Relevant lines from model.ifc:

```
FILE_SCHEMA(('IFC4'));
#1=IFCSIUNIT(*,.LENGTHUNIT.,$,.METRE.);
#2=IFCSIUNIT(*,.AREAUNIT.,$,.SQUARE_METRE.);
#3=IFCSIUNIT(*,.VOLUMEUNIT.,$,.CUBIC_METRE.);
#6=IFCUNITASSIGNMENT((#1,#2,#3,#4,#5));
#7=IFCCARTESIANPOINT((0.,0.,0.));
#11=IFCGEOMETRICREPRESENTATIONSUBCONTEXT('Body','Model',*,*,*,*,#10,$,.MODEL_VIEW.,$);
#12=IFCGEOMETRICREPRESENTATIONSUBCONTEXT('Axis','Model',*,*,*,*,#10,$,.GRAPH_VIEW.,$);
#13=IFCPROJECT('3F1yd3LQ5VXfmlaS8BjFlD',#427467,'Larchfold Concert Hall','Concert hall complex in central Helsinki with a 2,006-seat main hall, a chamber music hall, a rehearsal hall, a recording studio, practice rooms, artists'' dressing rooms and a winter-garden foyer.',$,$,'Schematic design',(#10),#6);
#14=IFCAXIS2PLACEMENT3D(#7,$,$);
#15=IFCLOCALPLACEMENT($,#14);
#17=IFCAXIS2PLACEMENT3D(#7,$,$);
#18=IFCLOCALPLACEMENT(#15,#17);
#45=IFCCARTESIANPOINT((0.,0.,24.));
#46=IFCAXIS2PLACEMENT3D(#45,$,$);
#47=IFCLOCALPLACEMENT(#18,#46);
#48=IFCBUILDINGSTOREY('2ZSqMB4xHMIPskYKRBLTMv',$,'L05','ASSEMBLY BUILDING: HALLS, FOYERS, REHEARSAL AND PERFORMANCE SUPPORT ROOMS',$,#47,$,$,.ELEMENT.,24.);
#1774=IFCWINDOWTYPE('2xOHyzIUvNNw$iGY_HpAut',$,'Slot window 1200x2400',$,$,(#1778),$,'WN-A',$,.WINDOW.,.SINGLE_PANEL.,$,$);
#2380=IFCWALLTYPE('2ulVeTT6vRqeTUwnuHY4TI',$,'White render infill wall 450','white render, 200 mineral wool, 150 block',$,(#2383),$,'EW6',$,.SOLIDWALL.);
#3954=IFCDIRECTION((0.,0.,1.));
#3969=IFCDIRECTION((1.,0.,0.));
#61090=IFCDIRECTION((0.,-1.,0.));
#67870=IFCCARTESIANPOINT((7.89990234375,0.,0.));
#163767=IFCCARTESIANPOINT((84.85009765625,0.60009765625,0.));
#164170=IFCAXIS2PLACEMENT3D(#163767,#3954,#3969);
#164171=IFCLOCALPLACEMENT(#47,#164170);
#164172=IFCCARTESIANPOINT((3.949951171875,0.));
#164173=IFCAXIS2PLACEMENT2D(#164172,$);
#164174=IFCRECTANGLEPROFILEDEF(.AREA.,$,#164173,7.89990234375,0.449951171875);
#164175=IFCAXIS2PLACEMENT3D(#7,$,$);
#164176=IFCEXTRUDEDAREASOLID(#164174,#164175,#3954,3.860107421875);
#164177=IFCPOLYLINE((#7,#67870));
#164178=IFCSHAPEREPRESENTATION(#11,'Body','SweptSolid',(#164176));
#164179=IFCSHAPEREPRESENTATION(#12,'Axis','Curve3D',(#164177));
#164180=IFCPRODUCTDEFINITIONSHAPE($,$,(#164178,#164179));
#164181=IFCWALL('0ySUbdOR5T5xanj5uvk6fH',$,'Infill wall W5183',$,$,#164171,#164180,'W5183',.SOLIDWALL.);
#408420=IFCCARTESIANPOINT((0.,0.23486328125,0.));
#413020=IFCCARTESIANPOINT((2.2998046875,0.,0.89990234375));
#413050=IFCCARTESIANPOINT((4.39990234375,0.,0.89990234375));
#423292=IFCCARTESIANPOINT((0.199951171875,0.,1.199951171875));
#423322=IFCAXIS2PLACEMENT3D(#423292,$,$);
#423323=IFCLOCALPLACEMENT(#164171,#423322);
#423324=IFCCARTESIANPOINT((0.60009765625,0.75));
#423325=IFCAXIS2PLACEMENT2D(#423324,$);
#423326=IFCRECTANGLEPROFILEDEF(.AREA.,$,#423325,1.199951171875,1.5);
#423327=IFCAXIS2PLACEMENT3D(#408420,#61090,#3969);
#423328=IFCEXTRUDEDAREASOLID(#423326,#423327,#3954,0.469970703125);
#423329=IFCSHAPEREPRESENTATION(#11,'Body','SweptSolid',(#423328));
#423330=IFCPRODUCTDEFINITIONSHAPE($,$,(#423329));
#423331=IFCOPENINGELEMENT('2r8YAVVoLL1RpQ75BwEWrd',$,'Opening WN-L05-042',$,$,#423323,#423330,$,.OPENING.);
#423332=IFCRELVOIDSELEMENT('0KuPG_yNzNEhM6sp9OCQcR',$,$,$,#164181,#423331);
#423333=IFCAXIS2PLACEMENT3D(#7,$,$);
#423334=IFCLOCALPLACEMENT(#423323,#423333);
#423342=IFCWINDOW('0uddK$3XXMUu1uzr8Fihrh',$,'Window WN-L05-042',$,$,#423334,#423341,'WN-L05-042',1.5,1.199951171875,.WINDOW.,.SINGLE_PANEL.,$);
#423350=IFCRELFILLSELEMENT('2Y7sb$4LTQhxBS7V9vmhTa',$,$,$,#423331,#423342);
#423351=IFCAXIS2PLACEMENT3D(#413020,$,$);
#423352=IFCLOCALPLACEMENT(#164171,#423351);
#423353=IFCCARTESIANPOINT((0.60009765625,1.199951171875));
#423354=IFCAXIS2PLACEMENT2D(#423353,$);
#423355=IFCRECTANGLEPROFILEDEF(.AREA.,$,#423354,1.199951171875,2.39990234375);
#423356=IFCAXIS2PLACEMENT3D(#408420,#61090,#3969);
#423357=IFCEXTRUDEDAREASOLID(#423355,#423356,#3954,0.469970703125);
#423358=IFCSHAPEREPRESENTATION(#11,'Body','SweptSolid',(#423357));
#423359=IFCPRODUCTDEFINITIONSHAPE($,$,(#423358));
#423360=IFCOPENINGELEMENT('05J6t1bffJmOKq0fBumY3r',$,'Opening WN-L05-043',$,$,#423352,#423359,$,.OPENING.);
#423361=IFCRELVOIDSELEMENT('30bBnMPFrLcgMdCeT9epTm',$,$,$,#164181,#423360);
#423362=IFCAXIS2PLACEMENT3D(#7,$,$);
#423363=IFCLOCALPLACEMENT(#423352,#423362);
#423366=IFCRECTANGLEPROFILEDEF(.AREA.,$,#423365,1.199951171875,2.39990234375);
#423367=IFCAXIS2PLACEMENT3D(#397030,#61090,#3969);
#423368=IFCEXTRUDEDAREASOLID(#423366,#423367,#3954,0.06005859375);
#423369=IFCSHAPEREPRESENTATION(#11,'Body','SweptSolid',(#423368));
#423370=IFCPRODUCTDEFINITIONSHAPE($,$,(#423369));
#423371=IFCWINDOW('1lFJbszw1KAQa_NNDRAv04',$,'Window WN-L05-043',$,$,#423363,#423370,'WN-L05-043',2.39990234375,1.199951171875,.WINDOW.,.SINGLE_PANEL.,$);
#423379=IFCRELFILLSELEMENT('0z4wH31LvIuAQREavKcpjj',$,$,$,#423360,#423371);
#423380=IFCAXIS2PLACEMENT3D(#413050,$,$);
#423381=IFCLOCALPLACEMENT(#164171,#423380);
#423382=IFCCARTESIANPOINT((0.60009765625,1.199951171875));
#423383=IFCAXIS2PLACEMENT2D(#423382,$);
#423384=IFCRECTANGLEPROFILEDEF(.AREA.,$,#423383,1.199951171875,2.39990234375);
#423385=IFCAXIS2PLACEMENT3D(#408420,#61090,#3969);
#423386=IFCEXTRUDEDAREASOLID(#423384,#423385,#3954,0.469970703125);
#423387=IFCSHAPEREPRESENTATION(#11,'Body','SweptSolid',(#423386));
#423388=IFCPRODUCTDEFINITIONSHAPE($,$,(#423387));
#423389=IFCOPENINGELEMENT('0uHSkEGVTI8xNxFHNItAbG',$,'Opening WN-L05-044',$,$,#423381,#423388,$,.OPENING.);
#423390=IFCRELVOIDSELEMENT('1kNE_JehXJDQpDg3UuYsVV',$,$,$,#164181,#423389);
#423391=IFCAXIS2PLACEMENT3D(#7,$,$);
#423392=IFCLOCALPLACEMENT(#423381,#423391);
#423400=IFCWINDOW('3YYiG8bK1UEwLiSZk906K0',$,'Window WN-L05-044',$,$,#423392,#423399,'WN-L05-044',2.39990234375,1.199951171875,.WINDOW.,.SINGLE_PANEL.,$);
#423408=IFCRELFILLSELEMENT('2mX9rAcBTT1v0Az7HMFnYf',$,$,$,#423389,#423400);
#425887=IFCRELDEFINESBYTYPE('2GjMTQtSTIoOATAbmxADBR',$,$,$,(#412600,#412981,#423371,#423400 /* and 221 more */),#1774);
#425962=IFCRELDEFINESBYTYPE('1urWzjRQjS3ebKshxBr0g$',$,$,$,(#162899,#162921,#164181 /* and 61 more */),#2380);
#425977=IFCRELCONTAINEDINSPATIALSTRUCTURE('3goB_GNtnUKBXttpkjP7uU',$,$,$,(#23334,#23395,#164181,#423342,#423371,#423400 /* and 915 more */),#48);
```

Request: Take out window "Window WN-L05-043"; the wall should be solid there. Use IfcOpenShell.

```python
import ifcopenshell
import ifcopenshell.api.feature
import ifcopenshell.api.root
import ifcopenshell.geom
import ifcopenshell.util.shape

model = ifcopenshell.open("model.ifc")
settings = ifcopenshell.geom.settings()


def volume(element):
    """Net volume in cubic metres, openings subtracted."""
    shape = ifcopenshell.geom.create_shape(settings, element)
    return ifcopenshell.util.shape.get_volume(shape.geometry)


window = model.by_guid("1lFJbszw1KAQa_NNDRAv04")
opening = window.FillsVoids[0].RelatingOpeningElement
wall = opening.VoidsElements[0].RelatingBuildingElement
before = volume(wall)

ifcopenshell.api.root.remove_product(model, product=window)
ifcopenshell.api.feature.remove_feature(model, feature=opening)

after = volume(wall)

print(f"wall volume {before:.3f} -> {after:.3f} m3")

model.write("model_edited.ifc")
```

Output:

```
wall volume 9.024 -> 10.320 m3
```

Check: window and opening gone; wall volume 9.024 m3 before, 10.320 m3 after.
